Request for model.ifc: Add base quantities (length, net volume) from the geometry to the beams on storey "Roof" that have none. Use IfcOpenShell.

First a look at what the model holds.

```python
import ifcopenshell
import ifcopenshell.util.element
import ifcopenshell.util.unit

model = ifcopenshell.open("model.ifc")
print(model.schema)
for unit_type in ("LENGTHUNIT", "AREAUNIT", "VOLUMEUNIT"):
    print(unit_type, ifcopenshell.util.unit.calculate_unit_scale(model, unit_type))
storey = next(s for s in model.by_type("IfcBuildingStorey") if s.Name == "Roof")
beams = [e for e in ifcopenshell.util.element.get_decomposition(storey) if e.is_a("IfcBeam")]
for e in sorted(beams, key=lambda e: e.id()):
    print(e.id(), e.is_a(), e.Name, list(ifcopenshell.util.element.get_psets(e, qtos_only=True)), sep=" | ")
```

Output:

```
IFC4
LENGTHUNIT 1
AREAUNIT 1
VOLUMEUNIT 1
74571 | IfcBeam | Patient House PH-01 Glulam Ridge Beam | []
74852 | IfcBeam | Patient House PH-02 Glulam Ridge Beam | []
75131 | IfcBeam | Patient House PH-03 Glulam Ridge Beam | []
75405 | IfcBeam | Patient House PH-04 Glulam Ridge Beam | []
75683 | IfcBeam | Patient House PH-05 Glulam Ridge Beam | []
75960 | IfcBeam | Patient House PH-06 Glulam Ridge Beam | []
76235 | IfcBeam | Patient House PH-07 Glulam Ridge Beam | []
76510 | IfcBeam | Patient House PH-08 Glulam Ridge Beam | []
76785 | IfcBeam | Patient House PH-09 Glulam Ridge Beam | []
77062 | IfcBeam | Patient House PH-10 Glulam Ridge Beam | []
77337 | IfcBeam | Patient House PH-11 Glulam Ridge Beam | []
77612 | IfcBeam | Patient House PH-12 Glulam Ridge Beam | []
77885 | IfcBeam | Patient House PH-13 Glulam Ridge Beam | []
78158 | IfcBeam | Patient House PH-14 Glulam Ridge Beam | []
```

```python
import ifcopenshell
import ifcopenshell.api.pset
import ifcopenshell.geom
import ifcopenshell.util.element
import ifcopenshell.util.shape
import ifcopenshell.util.unit

model = ifcopenshell.open("model.ifc")
unit_scale = ifcopenshell.util.unit.calculate_unit_scale(model)
volume_scale = ifcopenshell.util.unit.calculate_unit_scale(model, "VOLUMEUNIT")
settings = ifcopenshell.geom.settings()

storey = next(s for s in model.by_type("IfcBuildingStorey") if s.Name == "Roof")
beams = [e for e in ifcopenshell.util.element.get_decomposition(storey) if e.is_a("IfcBeam")]

for e in sorted(beams, key=lambda e: e.id()):
    if ifcopenshell.util.element.get_psets(e, qtos_only=True, should_inherit=False):
        continue
    # Geometry comes back in metres, in the element's own axes.
    shape = ifcopenshell.geom.create_shape(settings, e)
    values = {
        "Length": ifcopenshell.util.shape.get_max_xyz(shape.geometry) / unit_scale,
        "NetVolume": ifcopenshell.util.shape.get_volume(shape.geometry) / volume_scale,
    }
    qto = ifcopenshell.api.pset.add_qto(model, product=e, name="Qto_BeamBaseQuantities")
    ifcopenshell.api.pset.edit_qto(model, qto=qto, properties=values)
    print(e.id(), {k: round(v, 3) for k, v in values.items()})

model.write("model_edited.ifc")
```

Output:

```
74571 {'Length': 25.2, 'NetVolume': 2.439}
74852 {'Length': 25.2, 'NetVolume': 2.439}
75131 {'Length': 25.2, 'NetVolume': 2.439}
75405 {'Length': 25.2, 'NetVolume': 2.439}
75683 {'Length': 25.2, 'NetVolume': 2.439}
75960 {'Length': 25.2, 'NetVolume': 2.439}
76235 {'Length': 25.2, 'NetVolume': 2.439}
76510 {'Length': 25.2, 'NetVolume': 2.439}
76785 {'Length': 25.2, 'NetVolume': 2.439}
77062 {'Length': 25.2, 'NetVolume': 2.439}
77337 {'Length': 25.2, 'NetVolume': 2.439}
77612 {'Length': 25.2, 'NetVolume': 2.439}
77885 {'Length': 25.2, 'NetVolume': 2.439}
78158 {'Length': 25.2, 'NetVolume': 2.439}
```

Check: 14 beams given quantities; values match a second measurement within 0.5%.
